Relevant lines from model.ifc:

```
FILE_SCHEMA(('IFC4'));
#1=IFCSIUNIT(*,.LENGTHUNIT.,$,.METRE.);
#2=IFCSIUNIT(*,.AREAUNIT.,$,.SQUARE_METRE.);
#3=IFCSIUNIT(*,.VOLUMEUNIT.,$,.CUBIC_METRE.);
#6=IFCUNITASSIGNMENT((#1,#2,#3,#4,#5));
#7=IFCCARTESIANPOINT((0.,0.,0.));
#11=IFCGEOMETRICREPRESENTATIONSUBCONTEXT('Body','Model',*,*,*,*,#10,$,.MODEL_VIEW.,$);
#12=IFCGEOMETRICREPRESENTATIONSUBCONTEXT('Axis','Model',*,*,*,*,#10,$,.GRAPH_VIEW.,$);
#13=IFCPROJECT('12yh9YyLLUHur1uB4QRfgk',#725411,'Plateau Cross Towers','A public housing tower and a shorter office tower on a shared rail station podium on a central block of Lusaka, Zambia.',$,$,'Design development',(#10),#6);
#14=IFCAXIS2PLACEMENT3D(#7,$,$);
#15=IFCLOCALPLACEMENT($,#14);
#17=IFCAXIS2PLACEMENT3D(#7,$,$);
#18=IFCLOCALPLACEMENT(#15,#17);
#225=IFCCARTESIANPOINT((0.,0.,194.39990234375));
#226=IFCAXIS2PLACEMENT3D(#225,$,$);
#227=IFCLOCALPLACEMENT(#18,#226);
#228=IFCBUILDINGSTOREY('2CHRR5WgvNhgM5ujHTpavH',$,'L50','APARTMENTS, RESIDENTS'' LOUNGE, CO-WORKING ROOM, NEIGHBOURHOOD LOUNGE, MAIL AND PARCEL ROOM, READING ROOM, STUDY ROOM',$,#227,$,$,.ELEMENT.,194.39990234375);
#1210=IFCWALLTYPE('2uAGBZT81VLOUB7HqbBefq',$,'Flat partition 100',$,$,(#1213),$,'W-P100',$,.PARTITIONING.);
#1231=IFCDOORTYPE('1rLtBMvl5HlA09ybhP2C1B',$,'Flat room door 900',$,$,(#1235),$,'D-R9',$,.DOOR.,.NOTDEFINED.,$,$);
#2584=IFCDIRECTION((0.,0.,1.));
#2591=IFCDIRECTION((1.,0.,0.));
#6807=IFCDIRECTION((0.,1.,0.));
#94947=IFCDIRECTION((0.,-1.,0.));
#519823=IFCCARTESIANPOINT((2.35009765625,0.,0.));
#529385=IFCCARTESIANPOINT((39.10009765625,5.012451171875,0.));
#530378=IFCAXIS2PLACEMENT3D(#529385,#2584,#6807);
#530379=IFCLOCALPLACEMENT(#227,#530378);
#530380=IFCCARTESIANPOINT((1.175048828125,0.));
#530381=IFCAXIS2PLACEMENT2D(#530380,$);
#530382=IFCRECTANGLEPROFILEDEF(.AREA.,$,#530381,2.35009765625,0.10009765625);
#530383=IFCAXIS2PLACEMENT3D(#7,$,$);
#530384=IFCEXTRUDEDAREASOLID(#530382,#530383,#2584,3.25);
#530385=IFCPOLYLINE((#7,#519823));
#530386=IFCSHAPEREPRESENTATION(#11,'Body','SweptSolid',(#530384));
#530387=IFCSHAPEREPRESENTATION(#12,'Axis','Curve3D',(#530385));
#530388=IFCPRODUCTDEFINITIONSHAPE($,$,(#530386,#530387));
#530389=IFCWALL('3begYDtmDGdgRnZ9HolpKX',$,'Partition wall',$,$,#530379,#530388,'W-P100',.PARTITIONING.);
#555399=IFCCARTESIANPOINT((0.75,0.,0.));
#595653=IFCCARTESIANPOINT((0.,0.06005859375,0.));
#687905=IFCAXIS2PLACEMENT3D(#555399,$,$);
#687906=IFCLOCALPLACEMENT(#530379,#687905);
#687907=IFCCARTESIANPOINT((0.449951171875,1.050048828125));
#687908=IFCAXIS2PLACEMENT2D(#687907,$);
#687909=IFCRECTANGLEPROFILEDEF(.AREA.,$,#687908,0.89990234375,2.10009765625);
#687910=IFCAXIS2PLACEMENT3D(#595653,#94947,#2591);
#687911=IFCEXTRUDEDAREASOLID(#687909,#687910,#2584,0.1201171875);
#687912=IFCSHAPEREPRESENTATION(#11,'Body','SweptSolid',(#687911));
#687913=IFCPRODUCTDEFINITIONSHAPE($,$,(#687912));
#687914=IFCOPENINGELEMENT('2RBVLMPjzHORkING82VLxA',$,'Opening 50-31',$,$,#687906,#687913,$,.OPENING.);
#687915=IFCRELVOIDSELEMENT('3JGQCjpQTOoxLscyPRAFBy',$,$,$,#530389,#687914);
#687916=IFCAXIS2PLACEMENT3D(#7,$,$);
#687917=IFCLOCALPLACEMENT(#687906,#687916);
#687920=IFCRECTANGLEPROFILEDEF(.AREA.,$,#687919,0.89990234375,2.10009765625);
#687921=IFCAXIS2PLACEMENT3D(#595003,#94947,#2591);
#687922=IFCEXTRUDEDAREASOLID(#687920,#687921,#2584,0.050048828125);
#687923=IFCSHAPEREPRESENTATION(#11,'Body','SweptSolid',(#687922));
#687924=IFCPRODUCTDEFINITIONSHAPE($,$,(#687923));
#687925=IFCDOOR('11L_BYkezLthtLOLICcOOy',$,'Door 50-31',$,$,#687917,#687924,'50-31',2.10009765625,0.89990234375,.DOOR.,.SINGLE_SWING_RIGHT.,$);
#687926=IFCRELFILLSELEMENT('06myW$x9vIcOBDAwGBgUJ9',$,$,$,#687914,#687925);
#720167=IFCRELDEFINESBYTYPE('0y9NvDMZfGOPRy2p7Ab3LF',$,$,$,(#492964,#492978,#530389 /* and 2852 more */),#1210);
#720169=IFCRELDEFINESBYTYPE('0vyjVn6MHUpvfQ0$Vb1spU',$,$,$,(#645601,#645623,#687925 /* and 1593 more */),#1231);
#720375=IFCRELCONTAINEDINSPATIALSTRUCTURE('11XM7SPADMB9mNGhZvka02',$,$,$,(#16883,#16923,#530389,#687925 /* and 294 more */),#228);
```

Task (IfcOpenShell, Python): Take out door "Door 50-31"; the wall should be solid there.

```python
import ifcopenshell
import ifcopenshell.api.feature
import ifcopenshell.api.root
import ifcopenshell.geom
import ifcopenshell.util.shape

model = ifcopenshell.open("model.ifc")
settings = ifcopenshell.geom.settings()


def volume(element):
    """Net volume in cubic metres, openings subtracted."""
    shape = ifcopenshell.geom.create_shape(settings, element)
    return ifcopenshell.util.shape.get_volume(shape.geometry)


door = model.by_id(687925)
opening = door.FillsVoids[0].RelatingOpeningElement
wall = opening.VoidsElements[0].RelatingBuildingElement
before = volume(wall)

ifcopenshell.api.root.remove_product(model, product=door)
ifcopenshell.api.feature.remove_feature(model, feature=opening)

after = volume(wall)

print(f"wall volume {before:.3f} -> {after:.3f} m3")

model.write("model_rev.ifc")
```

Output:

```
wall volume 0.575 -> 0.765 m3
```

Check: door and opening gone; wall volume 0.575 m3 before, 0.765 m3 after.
